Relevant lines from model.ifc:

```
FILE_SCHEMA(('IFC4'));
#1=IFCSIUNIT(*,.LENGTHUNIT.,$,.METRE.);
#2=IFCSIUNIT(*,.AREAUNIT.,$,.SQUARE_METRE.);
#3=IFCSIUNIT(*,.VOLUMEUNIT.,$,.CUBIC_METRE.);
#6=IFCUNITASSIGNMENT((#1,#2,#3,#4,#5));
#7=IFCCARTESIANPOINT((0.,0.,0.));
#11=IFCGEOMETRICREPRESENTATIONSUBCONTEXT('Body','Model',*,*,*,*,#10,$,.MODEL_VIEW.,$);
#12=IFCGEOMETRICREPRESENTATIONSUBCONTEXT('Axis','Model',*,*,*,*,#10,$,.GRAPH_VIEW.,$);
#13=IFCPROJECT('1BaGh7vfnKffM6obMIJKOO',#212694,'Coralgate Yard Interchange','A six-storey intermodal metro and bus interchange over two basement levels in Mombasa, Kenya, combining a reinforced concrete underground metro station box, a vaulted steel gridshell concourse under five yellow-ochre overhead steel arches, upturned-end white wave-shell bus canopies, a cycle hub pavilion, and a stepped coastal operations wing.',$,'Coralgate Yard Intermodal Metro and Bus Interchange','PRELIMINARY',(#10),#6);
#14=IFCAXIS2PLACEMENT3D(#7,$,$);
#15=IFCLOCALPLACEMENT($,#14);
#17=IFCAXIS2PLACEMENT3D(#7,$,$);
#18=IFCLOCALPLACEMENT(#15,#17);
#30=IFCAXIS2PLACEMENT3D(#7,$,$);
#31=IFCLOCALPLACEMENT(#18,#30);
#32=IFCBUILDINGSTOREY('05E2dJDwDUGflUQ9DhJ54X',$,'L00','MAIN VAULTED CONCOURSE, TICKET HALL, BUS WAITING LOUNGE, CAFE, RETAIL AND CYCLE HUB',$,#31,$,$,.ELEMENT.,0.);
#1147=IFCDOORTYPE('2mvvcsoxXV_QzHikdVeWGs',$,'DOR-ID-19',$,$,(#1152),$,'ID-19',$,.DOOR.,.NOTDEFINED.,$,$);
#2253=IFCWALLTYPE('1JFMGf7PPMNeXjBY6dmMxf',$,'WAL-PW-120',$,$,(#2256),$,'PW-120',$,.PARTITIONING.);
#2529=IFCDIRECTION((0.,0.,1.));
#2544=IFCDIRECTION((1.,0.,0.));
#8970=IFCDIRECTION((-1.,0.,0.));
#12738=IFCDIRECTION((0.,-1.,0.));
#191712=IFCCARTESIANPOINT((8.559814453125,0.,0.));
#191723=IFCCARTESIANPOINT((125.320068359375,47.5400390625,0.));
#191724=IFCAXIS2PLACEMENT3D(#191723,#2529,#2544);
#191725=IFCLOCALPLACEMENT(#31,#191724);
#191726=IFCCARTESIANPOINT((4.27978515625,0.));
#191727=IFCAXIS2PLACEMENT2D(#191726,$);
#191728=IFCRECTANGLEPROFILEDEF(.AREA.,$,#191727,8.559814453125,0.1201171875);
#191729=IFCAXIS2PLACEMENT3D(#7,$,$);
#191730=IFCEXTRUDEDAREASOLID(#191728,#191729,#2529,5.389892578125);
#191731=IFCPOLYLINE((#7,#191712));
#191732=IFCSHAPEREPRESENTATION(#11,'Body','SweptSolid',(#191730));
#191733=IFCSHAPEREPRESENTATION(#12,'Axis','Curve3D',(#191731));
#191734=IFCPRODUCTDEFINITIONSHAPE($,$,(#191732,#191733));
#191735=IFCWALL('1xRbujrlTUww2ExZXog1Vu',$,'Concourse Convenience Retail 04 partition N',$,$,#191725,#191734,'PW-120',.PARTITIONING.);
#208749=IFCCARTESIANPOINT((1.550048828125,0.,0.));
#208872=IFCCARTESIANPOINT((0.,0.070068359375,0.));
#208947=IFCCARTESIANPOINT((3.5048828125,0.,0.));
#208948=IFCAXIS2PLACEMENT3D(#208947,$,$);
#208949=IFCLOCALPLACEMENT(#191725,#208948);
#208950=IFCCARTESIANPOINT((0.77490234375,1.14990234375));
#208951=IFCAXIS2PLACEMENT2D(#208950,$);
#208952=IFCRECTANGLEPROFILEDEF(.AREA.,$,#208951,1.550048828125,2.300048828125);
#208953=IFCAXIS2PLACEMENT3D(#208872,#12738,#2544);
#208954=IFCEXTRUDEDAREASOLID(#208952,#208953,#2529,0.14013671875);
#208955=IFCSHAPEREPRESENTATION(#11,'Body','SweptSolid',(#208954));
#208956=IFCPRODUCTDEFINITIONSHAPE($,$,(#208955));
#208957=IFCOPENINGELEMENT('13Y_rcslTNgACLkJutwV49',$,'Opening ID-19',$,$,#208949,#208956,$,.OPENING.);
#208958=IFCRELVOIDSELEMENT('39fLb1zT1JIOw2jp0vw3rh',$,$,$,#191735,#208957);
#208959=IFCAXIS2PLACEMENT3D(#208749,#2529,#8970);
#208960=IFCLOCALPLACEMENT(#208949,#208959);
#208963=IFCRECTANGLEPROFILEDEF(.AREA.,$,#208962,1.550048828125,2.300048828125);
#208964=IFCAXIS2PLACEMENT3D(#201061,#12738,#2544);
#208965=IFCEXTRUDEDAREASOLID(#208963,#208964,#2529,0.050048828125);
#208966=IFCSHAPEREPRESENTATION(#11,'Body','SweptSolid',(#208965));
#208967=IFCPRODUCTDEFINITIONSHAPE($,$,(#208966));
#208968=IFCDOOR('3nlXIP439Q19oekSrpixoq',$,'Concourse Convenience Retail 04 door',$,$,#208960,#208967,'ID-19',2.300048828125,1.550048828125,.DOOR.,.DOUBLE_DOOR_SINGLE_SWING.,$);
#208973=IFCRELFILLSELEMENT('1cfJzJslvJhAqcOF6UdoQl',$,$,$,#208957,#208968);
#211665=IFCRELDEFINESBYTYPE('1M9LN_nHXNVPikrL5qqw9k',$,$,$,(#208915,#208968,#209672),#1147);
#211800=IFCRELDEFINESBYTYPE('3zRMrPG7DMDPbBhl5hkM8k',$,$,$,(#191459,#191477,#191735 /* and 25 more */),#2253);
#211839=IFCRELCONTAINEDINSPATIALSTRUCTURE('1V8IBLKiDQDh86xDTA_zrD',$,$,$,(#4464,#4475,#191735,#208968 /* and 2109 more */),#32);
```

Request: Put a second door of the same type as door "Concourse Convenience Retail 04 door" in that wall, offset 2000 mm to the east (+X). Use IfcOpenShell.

```python
import ifcopenshell
import ifcopenshell.api.feature
import ifcopenshell.api.geometry
import ifcopenshell.api.root
import ifcopenshell.geom
import ifcopenshell.util.element
import ifcopenshell.util.placement
import ifcopenshell.util.shape
import ifcopenshell.util.unit

model = ifcopenshell.open("model.ifc")
unit_scale = ifcopenshell.util.unit.calculate_unit_scale(model)
settings = ifcopenshell.geom.settings()


def volume(element):
    """Net volume in cubic metres, openings subtracted."""
    shape = ifcopenshell.geom.create_shape(settings, element)
    return ifcopenshell.util.shape.get_volume(shape.geometry)


door = model.by_guid("3nlXIP439Q19oekSrpixoq")
opening = door.FillsVoids[0].RelatingOpeningElement
wall = opening.VoidsElements[0].RelatingBuildingElement
before = volume(wall)
shift = ifcopenshell.util.placement.get_local_placement(wall.ObjectPlacement)[:3, 0] * 2 / unit_scale

# copy_class copies the void relationship, type, container and properties, but no geometry.
new_opening = ifcopenshell.api.root.copy_class(model, product=opening)
new_opening.Representation = ifcopenshell.util.element.copy_deep(
    model, opening.Representation, exclude=["IfcGeometricRepresentationContext", "IfcRepresentationMap"]
)
new_door = ifcopenshell.api.root.copy_class(model, product=door)
new_door.Representation = ifcopenshell.util.element.copy_deep(
    model, door.Representation, exclude=["IfcGeometricRepresentationContext", "IfcRepresentationMap"]
)
new_door.Tag = None
ifcopenshell.api.feature.add_filling(model, opening=new_opening, element=new_door)

for old, new in ((opening, new_opening), (door, new_door)):
    matrix = ifcopenshell.util.placement.get_local_placement(old.ObjectPlacement)
    matrix[:3, 3] += shift
    ifcopenshell.api.geometry.edit_object_placement(model, product=new, matrix=matrix, is_si=False)

after = volume(wall)

print(f"wall volume {before:.3f} -> {after:.3f} m3")

model.write("model_edited.ifc")
```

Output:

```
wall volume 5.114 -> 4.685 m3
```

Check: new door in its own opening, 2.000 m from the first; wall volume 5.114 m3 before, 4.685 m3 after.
